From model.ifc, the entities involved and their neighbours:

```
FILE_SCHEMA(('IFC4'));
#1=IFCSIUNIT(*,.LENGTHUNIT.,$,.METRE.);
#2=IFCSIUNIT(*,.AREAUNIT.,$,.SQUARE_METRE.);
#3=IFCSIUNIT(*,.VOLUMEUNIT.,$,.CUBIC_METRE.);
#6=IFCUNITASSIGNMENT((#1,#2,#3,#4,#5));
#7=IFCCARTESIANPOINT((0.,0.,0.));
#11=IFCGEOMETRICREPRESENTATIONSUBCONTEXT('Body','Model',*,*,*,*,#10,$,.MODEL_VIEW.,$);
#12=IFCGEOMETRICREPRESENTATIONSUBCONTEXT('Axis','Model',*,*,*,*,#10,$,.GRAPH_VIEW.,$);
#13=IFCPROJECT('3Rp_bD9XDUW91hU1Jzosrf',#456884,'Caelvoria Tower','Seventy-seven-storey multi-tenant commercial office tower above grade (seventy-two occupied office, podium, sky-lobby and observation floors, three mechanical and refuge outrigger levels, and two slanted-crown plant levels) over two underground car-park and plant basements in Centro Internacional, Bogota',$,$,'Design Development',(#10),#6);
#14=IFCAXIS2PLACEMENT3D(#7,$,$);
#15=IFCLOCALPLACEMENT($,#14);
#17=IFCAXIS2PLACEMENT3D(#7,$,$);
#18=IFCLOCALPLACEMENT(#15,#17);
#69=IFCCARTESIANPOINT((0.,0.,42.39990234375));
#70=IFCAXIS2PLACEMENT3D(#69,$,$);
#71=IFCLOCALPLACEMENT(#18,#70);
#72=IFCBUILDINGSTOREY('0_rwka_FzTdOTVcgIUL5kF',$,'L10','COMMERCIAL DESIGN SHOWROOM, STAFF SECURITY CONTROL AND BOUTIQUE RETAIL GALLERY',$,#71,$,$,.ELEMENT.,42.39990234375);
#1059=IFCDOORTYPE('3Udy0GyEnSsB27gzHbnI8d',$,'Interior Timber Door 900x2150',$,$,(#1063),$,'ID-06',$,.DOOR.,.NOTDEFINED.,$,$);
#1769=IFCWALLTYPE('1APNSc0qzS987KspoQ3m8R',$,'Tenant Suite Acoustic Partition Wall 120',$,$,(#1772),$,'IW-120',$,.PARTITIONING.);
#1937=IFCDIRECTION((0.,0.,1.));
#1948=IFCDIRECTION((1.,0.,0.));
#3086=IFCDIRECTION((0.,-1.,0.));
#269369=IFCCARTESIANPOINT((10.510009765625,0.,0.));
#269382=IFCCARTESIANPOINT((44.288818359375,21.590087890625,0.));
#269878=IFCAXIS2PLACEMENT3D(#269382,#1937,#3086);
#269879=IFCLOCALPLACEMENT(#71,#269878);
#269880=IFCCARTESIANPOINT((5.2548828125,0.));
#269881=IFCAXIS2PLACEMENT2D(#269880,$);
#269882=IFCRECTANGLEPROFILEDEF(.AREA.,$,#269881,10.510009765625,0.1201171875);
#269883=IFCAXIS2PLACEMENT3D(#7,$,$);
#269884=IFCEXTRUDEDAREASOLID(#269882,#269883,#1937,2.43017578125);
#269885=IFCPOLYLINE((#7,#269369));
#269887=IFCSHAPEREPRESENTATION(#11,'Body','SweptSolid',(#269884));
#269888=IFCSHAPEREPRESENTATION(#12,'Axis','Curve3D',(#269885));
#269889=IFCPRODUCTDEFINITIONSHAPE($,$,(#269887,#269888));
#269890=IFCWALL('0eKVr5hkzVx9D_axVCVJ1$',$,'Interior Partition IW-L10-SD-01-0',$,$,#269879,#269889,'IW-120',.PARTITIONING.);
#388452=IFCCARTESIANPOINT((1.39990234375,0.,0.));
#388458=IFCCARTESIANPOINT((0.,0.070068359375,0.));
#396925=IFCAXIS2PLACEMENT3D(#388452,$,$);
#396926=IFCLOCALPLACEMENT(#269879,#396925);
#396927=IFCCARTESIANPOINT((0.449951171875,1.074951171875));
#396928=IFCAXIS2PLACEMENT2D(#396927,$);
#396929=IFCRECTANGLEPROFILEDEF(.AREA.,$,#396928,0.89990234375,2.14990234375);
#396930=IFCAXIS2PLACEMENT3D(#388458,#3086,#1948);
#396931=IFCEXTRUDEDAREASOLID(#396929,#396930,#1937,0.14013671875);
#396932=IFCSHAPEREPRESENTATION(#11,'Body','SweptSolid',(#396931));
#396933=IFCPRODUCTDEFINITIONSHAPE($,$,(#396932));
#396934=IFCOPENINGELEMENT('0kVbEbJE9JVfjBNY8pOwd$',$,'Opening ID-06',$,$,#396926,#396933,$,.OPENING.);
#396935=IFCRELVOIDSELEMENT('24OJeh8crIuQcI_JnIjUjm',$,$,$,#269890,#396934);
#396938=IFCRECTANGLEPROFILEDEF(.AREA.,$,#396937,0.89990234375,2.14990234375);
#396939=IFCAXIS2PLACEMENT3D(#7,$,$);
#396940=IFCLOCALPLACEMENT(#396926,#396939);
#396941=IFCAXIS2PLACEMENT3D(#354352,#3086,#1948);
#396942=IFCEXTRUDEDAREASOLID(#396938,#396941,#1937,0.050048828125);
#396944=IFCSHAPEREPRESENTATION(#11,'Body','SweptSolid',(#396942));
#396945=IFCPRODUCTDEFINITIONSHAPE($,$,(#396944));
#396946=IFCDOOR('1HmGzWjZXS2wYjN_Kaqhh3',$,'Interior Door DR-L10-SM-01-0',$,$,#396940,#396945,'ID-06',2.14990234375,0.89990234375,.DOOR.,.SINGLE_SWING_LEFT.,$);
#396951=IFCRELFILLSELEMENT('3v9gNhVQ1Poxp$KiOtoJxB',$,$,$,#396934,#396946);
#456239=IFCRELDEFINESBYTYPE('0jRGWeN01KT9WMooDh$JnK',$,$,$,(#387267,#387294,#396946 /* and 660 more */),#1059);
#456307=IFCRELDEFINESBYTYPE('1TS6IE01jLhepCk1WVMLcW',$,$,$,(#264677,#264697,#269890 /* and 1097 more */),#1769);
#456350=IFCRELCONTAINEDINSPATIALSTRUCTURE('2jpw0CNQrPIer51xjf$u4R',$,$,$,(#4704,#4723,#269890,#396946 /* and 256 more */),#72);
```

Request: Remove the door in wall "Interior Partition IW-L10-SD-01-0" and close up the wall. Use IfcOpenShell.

```python
import ifcopenshell
import ifcopenshell.api.feature
import ifcopenshell.api.root
import ifcopenshell.geom
import ifcopenshell.util.shape

model = ifcopenshell.open("model.ifc")
settings = ifcopenshell.geom.settings()


def volume(element):
    """Net volume in cubic metres, openings subtracted."""
    shape = ifcopenshell.geom.create_shape(settings, element)
    return ifcopenshell.util.shape.get_volume(shape.geometry)


door = model.by_id(396946)
opening = door.FillsVoids[0].RelatingOpeningElement
wall = opening.VoidsElements[0].RelatingBuildingElement
before = volume(wall)

ifcopenshell.api.root.remove_product(model, product=door)
ifcopenshell.api.feature.remove_feature(model, feature=opening)

after = volume(wall)

print(f"wall volume {before:.3f} -> {after:.3f} m3")

model.write("model_edited.ifc")
```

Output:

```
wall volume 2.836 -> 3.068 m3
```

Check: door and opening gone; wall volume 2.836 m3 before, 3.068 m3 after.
